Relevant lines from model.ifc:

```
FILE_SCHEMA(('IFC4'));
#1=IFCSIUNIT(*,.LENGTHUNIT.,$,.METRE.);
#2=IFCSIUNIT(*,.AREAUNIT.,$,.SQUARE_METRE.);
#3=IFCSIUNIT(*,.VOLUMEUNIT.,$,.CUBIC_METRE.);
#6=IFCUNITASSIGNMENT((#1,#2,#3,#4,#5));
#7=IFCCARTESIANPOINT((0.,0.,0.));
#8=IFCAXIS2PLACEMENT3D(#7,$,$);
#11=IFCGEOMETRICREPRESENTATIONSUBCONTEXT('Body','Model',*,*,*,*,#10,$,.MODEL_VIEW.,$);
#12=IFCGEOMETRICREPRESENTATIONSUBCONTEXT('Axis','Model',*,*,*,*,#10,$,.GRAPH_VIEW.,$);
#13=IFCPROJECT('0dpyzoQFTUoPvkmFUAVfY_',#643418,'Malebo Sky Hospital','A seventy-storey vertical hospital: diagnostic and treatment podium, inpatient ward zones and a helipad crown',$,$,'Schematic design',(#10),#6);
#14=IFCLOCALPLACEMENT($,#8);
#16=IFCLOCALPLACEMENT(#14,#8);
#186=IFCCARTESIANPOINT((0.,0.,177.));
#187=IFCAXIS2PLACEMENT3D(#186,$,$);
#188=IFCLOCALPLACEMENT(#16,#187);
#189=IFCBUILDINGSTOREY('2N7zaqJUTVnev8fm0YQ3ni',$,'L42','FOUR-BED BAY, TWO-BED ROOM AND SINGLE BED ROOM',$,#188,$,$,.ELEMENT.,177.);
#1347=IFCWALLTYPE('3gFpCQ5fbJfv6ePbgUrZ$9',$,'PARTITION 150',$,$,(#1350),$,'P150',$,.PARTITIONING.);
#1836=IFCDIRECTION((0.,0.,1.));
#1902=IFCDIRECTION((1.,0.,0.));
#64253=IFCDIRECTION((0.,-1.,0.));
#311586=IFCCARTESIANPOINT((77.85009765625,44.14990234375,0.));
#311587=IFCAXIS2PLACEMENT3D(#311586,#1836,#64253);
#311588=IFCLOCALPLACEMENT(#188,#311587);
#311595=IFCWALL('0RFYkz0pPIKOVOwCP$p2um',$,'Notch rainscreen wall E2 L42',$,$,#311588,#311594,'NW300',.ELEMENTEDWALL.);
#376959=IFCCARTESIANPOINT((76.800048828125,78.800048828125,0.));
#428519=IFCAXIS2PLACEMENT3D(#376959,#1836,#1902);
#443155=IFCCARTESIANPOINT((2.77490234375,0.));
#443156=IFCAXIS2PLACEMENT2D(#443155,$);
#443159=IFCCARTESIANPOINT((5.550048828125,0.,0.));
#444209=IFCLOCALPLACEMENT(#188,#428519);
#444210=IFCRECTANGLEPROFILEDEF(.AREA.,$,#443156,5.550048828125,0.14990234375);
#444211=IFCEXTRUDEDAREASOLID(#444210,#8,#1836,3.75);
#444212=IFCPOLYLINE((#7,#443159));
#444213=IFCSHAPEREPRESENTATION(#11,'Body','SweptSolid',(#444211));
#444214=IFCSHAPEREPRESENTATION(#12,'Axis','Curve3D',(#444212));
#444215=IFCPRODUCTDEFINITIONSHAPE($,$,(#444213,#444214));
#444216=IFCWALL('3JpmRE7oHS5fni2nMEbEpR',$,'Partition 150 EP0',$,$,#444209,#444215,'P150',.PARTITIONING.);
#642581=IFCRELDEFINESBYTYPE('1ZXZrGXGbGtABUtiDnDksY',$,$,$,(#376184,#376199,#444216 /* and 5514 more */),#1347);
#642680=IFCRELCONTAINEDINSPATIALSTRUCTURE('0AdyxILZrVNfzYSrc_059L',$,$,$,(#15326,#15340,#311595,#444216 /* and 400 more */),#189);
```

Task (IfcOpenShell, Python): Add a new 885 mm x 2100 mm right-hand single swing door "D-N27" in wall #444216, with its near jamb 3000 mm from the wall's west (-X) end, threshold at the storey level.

```python
import numpy as np
import ifcopenshell
import ifcopenshell.api.feature
import ifcopenshell.api.geometry
import ifcopenshell.api.root
import ifcopenshell.api.spatial
import ifcopenshell.geom
import ifcopenshell.util.element
import ifcopenshell.util.placement
import ifcopenshell.util.representation
import ifcopenshell.util.shape
import ifcopenshell.util.unit

model = ifcopenshell.open("model.ifc")
unit_scale = ifcopenshell.util.unit.calculate_unit_scale(model)
settings = ifcopenshell.geom.settings()


def volume(element):
    """Net volume in cubic metres, openings subtracted."""
    shape = ifcopenshell.geom.create_shape(settings, element)
    return ifcopenshell.util.shape.get_volume(shape.geometry)


wall = model.by_guid("3JpmRE7oHS5fni2nMEbEpR")
storey = ifcopenshell.util.element.get_container(wall, ifc_class="IfcBuildingStorey")
context = ifcopenshell.util.representation.get_context(model, "Model", "Body", "MODEL_VIEW")
before = volume(wall)

width, height, from_end, sill = 0.885, 2.1, 3, 0.0  # metres

# The wall runs along its own X axis, and the end named is its -X end.
wall_shape = ifcopenshell.geom.create_shape(settings, wall)
x, y, z = ifcopenshell.util.shape.get_vertices(wall_shape.geometry).T
start = x.min() + from_end
face, thickness = float(y.min()), float(y.max() - y.min())
wall_matrix = ifcopenshell.util.placement.get_local_placement(wall.ObjectPlacement)
level = ifcopenshell.util.placement.get_local_placement(storey.ObjectPlacement)[2, 3]


def in_wall(x, y):
    """Placement at x, y metres in the wall's axes, at sill height."""
    matrix = wall_matrix.copy()
    matrix[:, 3] = wall_matrix @ np.array([x / unit_scale, y / unit_scale, 0.0, 1.0])
    matrix[2, 3] = level + sill / unit_scale
    return matrix


# Opening: a box that overshoots both wall faces by 50 mm.
opening = ifcopenshell.api.root.create_entity(model, ifc_class="IfcOpeningElement", predefined_type="OPENING")
box = ifcopenshell.api.geometry.add_wall_representation(
    model, context=context, length=width, height=height, thickness=thickness + 0.1
)
ifcopenshell.api.geometry.assign_representation(model, product=opening, representation=box)
ifcopenshell.api.geometry.edit_object_placement(model, product=opening, matrix=in_wall(start, face - 0.05), is_si=False)
ifcopenshell.api.feature.add_feature(model, feature=opening, element=wall)

door = ifcopenshell.api.root.create_entity(model, ifc_class="IfcDoor", name="D-N27", predefined_type="DOOR")
door.OverallWidth, door.OverallHeight = width / unit_scale, height / unit_scale
door.OperationType = "SINGLE_SWING_RIGHT"
body = ifcopenshell.api.geometry.add_door_representation(
    model,
    context=context,
    overall_width=door.OverallWidth,
    overall_height=door.OverallHeight,
    operation_type="SINGLE_SWING_RIGHT",
    lining_properties={"LiningDepth": thickness / unit_scale, "ThresholdDepth": thickness / unit_scale},
)
ifcopenshell.api.geometry.assign_representation(model, product=door, representation=body)
ifcopenshell.api.spatial.assign_container(model, products=[door], relating_structure=storey)
ifcopenshell.api.feature.add_filling(model, opening=opening, element=door)

# The lining spans the wall, so the door starts at the wall face.
ifcopenshell.api.geometry.edit_object_placement(model, product=door, matrix=in_wall(start, face), is_si=False)

after = volume(wall)

print(f"wall volume {before:.3f} -> {after:.3f} m3")

model.write("model_v2.ifc")
```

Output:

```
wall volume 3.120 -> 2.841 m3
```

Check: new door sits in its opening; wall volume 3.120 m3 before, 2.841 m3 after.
